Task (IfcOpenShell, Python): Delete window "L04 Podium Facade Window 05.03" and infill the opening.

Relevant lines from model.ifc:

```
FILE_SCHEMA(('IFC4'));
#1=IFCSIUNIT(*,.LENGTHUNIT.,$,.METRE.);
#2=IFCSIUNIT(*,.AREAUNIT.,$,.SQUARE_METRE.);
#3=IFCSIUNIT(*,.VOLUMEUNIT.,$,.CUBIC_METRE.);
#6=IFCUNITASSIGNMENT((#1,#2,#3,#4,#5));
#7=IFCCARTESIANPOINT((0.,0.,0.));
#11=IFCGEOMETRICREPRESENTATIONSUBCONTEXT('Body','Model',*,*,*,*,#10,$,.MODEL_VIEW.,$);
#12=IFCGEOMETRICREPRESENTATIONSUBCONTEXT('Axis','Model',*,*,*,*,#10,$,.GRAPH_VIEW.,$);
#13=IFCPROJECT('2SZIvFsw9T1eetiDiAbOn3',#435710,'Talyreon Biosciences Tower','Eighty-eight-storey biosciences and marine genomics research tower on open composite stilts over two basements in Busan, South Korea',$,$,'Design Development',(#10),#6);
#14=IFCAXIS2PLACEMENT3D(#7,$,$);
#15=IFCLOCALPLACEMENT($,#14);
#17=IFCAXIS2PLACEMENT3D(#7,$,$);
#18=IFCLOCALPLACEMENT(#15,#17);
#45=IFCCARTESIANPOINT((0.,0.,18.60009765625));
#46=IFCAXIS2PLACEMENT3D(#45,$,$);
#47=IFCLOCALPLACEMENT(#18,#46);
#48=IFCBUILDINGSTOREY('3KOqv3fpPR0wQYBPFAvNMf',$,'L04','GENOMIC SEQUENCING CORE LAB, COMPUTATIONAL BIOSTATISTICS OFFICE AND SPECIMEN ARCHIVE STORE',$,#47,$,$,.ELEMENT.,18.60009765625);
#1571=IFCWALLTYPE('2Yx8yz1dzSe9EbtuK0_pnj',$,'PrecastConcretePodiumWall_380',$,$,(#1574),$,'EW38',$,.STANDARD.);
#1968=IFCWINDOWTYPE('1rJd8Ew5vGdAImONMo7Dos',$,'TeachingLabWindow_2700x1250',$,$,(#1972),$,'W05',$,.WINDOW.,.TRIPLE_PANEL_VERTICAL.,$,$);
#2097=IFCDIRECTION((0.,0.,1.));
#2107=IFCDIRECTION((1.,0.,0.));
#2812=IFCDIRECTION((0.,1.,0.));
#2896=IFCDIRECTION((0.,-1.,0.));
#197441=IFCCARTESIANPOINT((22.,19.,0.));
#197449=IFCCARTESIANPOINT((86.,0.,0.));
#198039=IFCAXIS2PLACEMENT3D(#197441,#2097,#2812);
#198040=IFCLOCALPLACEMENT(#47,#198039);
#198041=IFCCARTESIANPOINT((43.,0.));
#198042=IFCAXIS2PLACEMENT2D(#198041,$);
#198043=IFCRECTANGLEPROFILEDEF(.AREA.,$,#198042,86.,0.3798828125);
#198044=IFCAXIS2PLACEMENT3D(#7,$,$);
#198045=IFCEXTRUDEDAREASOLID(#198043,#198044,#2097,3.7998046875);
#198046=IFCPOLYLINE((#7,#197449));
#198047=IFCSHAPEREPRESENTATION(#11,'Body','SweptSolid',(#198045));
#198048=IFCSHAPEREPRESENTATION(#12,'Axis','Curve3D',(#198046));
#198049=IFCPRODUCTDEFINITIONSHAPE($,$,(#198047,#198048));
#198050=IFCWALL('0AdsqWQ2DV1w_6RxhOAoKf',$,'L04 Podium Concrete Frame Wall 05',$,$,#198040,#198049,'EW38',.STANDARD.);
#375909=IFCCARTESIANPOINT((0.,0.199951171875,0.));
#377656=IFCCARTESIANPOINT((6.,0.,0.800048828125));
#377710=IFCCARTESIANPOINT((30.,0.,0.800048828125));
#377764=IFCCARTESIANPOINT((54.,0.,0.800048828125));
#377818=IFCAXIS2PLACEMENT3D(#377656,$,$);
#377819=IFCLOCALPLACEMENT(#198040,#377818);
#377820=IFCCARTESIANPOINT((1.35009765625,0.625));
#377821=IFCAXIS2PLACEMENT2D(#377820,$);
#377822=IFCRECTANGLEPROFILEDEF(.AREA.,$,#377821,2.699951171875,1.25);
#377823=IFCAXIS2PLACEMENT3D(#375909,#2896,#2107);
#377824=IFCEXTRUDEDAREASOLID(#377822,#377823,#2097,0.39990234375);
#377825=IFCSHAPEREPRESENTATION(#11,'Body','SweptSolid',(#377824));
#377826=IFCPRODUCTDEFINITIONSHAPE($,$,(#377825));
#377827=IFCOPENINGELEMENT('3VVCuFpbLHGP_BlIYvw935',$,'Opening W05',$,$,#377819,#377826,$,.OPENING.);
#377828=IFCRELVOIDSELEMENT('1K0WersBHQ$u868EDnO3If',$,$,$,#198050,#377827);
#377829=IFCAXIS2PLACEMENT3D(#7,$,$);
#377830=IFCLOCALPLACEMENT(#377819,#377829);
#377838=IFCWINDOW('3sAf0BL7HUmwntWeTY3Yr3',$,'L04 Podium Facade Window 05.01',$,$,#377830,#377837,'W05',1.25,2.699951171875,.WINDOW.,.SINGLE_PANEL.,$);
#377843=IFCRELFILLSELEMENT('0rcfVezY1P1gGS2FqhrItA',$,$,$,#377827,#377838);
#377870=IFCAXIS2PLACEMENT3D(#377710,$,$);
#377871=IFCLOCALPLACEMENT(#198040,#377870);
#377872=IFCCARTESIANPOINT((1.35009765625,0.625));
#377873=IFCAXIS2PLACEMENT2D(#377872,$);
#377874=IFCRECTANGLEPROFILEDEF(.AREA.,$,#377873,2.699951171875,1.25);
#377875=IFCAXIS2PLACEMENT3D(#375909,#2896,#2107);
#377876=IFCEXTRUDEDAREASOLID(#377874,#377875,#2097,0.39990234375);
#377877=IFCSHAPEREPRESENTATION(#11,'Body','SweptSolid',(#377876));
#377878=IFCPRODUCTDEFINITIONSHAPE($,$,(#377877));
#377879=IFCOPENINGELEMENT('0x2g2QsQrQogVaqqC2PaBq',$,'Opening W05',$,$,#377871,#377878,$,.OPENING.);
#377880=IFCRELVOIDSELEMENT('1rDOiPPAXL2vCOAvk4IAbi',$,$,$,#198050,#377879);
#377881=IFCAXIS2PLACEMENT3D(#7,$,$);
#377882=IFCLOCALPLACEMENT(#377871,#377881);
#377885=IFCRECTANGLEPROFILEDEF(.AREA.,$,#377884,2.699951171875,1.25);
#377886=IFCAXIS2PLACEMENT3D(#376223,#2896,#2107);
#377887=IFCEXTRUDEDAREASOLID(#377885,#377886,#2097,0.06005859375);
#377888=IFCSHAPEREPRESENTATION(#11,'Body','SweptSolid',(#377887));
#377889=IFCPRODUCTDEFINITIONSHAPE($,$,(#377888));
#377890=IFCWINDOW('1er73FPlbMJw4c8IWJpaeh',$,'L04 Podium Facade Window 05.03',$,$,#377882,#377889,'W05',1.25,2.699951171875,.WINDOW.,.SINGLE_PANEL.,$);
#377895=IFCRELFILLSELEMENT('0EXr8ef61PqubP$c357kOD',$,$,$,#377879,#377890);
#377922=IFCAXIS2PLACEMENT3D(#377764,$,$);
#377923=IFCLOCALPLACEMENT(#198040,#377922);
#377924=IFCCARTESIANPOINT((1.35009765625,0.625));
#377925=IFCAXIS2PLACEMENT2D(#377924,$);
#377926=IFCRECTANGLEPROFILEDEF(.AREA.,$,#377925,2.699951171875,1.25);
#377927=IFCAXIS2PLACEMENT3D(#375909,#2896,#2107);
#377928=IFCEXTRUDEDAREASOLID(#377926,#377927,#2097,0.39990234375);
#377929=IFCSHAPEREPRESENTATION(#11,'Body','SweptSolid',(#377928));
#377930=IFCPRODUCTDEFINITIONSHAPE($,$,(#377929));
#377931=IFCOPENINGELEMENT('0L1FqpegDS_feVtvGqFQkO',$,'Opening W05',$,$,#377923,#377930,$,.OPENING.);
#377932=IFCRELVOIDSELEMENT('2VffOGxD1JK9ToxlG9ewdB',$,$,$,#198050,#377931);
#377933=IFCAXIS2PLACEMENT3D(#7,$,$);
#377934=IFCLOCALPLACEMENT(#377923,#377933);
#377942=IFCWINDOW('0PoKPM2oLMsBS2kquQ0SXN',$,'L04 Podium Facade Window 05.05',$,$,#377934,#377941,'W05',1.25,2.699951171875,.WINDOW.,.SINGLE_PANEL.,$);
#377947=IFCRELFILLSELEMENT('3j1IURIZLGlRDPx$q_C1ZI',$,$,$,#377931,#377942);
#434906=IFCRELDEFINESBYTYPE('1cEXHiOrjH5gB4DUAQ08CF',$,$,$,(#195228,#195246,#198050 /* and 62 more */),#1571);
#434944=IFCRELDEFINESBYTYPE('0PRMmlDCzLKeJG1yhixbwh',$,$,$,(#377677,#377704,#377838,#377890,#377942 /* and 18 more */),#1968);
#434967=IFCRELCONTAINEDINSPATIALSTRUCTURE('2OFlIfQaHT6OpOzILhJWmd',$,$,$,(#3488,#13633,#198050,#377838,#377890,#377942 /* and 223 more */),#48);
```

```python
import ifcopenshell
import ifcopenshell.api.feature
import ifcopenshell.api.root
import ifcopenshell.geom
import ifcopenshell.util.shape

model = ifcopenshell.open("model.ifc")
settings = ifcopenshell.geom.settings()


def volume(element):
    """Net volume in cubic metres, openings subtracted."""
    shape = ifcopenshell.geom.create_shape(settings, element)
    return ifcopenshell.util.shape.get_volume(shape.geometry)


window = model.by_guid("1er73FPlbMJw4c8IWJpaeh")
opening = window.FillsVoids[0].RelatingOpeningElement
wall = opening.VoidsElements[0].RelatingBuildingElement
before = volume(wall)

ifcopenshell.api.root.remove_product(model, product=window)
ifcopenshell.api.feature.remove_feature(model, feature=opening)

after = volume(wall)

print(f"wall volume {before:.3f} -> {after:.3f} m3")

model.write("model_rev.ifc")
```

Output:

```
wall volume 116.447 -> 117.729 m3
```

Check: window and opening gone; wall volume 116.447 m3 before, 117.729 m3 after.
